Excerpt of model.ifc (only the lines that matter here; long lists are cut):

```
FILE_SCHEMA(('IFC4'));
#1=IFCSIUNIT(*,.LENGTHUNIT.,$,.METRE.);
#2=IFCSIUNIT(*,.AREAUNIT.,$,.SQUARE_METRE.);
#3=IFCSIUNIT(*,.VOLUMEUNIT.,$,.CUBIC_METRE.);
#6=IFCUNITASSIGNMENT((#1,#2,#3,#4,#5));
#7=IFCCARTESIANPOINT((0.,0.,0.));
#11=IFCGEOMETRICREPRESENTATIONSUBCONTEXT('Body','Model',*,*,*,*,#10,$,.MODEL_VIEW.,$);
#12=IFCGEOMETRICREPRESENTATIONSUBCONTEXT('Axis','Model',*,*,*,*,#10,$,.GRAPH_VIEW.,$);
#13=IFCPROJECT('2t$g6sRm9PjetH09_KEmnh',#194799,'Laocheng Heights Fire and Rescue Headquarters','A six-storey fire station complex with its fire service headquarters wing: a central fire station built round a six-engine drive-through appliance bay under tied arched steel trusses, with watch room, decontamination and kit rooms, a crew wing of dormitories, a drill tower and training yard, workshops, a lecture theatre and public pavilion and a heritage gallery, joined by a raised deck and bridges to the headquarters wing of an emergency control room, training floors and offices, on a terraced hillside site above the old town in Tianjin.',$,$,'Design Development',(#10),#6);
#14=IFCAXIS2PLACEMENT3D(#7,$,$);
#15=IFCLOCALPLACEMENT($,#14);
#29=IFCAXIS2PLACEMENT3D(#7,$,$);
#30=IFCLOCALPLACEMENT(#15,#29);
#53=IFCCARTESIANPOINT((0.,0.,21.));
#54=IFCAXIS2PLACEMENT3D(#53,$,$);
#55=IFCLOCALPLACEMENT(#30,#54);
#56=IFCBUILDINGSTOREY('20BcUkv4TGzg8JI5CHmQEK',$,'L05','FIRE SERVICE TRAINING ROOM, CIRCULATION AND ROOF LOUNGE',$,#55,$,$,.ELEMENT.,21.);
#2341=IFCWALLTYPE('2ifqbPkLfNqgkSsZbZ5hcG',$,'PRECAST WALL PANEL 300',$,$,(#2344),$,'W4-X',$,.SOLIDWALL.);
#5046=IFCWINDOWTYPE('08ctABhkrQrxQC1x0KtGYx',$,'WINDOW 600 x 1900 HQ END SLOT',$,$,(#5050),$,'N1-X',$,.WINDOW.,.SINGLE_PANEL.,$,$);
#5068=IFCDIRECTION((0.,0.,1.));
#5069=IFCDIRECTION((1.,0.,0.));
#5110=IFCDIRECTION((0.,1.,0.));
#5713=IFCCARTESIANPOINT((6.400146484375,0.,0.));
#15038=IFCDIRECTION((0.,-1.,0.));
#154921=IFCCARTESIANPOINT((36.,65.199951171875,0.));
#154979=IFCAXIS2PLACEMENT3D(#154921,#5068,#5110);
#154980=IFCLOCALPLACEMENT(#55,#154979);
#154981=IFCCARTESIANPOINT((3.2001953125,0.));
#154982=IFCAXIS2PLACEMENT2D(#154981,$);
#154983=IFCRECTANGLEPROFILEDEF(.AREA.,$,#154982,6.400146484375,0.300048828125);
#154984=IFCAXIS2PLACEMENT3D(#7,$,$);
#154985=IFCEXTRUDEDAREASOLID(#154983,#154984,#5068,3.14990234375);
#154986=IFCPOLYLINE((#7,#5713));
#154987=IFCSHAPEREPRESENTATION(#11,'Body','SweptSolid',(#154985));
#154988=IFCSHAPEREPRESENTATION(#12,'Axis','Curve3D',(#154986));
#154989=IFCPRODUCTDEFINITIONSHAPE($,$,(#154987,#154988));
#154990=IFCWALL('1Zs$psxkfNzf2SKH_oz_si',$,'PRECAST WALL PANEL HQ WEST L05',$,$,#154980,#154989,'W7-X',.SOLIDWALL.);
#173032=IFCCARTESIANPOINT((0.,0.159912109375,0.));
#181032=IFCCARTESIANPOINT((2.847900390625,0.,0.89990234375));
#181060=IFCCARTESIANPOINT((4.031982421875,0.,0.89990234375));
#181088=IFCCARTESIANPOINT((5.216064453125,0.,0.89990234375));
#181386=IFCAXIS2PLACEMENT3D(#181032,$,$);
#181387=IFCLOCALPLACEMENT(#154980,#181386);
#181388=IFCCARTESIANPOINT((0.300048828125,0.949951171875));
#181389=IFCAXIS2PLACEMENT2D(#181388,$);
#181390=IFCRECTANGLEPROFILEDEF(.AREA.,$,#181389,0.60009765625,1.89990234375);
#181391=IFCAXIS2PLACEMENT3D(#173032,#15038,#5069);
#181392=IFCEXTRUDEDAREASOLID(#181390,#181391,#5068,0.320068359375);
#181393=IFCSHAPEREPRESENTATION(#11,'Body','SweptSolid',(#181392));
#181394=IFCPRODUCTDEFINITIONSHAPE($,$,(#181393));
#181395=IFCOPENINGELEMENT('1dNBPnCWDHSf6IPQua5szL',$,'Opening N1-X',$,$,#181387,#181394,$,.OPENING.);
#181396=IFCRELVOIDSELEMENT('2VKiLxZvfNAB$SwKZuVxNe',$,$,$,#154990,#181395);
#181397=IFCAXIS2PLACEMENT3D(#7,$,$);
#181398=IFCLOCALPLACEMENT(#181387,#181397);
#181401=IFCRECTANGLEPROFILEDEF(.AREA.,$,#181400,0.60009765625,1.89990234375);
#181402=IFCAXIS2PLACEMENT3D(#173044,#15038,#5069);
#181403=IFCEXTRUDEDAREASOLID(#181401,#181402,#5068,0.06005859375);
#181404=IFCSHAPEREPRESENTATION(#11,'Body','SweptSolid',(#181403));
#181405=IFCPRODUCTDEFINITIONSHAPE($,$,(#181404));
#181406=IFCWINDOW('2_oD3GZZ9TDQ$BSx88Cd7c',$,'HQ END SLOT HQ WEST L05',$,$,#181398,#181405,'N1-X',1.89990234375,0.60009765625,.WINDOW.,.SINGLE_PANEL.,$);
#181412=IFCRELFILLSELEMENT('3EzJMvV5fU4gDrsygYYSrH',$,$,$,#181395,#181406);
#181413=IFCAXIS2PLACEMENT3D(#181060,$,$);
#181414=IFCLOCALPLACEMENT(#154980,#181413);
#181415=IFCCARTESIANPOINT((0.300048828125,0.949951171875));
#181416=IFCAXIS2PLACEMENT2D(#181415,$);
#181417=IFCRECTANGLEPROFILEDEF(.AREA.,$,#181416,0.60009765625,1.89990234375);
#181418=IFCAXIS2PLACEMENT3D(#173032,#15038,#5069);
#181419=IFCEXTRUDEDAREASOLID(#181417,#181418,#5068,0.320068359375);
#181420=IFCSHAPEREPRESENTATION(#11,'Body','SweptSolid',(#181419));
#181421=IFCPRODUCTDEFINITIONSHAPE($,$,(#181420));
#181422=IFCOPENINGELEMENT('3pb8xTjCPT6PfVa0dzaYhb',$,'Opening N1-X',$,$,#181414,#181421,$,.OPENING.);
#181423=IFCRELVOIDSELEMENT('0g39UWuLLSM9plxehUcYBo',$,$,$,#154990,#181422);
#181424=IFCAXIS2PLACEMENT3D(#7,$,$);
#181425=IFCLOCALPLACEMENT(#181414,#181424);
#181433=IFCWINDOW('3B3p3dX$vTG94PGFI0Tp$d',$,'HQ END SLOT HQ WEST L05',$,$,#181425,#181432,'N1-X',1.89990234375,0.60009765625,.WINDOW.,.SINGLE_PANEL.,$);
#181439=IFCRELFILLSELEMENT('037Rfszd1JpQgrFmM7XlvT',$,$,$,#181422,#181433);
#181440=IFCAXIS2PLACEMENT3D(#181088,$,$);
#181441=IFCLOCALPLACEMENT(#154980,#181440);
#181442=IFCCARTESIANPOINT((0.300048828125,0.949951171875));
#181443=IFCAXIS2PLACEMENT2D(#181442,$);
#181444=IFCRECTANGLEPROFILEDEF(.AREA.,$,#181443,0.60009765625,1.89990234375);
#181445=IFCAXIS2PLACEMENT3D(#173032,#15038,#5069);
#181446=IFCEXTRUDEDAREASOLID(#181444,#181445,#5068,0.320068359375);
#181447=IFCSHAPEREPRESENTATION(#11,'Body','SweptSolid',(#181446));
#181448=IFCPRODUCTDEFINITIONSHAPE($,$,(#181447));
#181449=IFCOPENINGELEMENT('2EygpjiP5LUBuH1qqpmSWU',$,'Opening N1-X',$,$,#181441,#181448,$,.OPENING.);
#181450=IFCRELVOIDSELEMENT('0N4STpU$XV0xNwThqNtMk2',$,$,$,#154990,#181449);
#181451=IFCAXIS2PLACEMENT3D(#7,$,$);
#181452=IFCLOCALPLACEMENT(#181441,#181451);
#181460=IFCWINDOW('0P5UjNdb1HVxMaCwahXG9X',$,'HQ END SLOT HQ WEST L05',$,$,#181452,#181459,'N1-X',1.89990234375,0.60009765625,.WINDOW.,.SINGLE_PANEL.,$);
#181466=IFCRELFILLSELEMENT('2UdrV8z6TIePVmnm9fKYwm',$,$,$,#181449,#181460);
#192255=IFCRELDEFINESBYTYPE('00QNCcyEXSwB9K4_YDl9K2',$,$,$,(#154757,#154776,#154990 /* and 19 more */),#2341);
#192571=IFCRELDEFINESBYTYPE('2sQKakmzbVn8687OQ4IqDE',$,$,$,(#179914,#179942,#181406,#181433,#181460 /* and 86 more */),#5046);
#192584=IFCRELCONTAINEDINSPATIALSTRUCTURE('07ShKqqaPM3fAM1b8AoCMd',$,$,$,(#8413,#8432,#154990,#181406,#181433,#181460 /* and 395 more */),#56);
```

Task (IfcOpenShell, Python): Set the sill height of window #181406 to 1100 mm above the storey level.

```python
import numpy as np
import ifcopenshell
import ifcopenshell.api.geometry
import ifcopenshell.geom
import ifcopenshell.util.element
import ifcopenshell.util.placement
import ifcopenshell.util.shape
import ifcopenshell.util.unit

model = ifcopenshell.open("model.ifc")
unit_scale = ifcopenshell.util.unit.calculate_unit_scale(model)

window = model.by_guid("2_oD3GZZ9TDQ$BSx88Cd7c")
opening = window.FillsVoids[0].RelatingOpeningElement
storey = ifcopenshell.util.element.get_container(window, ifc_class="IfcBuildingStorey")
level = ifcopenshell.util.placement.get_local_placement(storey.ObjectPlacement)[2, 3]

# The opening's origin need not be at the sill, so measure its lowest point.
shape = ifcopenshell.geom.create_shape(ifcopenshell.geom.settings(), opening)
bottom = ifcopenshell.util.shape.get_shape_bottom_elevation(shape, shape.geometry) / unit_scale
dz = level + 1.1 / unit_scale - bottom

shift = np.array([0.0, 0.0, dz])
# The window is placed relative to its opening, so it follows when the opening moves.
matrix = ifcopenshell.util.placement.get_local_placement(opening.ObjectPlacement)
matrix[:3, 3] += shift
ifcopenshell.api.geometry.edit_object_placement(
    model, product=opening, matrix=matrix, is_si=False, should_transform_children=True
)

print(f"moved by {dz * unit_scale:+.3f} m")

model.write("model_updated.ifc")
```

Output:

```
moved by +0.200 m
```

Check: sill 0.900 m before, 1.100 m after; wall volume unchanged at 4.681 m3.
